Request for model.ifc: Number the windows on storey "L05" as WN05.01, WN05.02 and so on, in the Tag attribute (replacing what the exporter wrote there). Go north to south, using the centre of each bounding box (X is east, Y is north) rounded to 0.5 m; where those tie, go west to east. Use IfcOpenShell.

First a look at what the model holds.

```python
import ifcopenshell
import ifcopenshell.util.element
import ifcopenshell.util.placement

model = ifcopenshell.open("model.ifc")
print(model.schema)
storey = next(s for s in model.by_type("IfcBuildingStorey") if s.Name == "L05")
windows = [e for e in ifcopenshell.util.element.get_decomposition(storey) if e.is_a("IfcWindow")]
for e in sorted(windows, key=lambda e: e.id()):
    origin = ifcopenshell.util.placement.get_local_placement(e.ObjectPlacement)[:3, 3]
    print(e.id(), e.Tag, e.Name, origin.round(2) + 0.0, sep=" | ")
```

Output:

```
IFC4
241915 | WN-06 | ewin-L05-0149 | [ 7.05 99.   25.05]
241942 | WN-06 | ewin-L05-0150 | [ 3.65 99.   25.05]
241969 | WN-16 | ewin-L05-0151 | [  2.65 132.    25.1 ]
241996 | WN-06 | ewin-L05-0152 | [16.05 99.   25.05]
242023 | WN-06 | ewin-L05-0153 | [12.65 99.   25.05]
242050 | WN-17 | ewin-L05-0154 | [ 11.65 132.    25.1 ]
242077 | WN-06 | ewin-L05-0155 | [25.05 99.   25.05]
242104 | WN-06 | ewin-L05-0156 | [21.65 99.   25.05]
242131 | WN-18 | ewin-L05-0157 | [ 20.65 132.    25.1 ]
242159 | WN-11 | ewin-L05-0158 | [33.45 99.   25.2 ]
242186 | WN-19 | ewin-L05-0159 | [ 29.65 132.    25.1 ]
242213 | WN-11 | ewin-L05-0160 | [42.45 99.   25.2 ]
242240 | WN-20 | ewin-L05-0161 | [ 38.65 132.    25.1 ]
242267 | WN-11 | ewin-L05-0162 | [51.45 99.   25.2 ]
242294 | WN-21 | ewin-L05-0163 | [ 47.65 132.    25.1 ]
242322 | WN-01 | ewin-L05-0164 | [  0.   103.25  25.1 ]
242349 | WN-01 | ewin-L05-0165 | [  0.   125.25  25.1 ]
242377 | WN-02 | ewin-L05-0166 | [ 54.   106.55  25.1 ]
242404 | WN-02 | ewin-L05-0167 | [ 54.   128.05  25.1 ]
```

```python
import ifcopenshell
import ifcopenshell.geom
import ifcopenshell.util.element
import ifcopenshell.util.shape

model = ifcopenshell.open("model.ifc")
settings = ifcopenshell.geom.settings()
settings.set("use-world-coords", True)


def centre(element):
    shape = ifcopenshell.geom.create_shape(settings, element)
    return ifcopenshell.util.shape.get_bbox_centroid(shape.geometry)


storey = next(s for s in model.by_type("IfcBuildingStorey") if s.Name == "L05")
windows = [e for e in ifcopenshell.util.element.get_decomposition(storey) if e.is_a("IfcWindow")]

# Insertion points can sit at a corner or the storey origin, so sort by the geometry (in metres).
centres = {e: centre(e) for e in windows}
windows.sort(key=lambda e: (-round(centres[e][1] / 0.5), centres[e][0]))

for i, e in enumerate(windows, start=1):
    number = f"WN05.{i:02d}"
    e.Tag = number
    print(e.id(), number)

model.write("model_rev.ifc")
```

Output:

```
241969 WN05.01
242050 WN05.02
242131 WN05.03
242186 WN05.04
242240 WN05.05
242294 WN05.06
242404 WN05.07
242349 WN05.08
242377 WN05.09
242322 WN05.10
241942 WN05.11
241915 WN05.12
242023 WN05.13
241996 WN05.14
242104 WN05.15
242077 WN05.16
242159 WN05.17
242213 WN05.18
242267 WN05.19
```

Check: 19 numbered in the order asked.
